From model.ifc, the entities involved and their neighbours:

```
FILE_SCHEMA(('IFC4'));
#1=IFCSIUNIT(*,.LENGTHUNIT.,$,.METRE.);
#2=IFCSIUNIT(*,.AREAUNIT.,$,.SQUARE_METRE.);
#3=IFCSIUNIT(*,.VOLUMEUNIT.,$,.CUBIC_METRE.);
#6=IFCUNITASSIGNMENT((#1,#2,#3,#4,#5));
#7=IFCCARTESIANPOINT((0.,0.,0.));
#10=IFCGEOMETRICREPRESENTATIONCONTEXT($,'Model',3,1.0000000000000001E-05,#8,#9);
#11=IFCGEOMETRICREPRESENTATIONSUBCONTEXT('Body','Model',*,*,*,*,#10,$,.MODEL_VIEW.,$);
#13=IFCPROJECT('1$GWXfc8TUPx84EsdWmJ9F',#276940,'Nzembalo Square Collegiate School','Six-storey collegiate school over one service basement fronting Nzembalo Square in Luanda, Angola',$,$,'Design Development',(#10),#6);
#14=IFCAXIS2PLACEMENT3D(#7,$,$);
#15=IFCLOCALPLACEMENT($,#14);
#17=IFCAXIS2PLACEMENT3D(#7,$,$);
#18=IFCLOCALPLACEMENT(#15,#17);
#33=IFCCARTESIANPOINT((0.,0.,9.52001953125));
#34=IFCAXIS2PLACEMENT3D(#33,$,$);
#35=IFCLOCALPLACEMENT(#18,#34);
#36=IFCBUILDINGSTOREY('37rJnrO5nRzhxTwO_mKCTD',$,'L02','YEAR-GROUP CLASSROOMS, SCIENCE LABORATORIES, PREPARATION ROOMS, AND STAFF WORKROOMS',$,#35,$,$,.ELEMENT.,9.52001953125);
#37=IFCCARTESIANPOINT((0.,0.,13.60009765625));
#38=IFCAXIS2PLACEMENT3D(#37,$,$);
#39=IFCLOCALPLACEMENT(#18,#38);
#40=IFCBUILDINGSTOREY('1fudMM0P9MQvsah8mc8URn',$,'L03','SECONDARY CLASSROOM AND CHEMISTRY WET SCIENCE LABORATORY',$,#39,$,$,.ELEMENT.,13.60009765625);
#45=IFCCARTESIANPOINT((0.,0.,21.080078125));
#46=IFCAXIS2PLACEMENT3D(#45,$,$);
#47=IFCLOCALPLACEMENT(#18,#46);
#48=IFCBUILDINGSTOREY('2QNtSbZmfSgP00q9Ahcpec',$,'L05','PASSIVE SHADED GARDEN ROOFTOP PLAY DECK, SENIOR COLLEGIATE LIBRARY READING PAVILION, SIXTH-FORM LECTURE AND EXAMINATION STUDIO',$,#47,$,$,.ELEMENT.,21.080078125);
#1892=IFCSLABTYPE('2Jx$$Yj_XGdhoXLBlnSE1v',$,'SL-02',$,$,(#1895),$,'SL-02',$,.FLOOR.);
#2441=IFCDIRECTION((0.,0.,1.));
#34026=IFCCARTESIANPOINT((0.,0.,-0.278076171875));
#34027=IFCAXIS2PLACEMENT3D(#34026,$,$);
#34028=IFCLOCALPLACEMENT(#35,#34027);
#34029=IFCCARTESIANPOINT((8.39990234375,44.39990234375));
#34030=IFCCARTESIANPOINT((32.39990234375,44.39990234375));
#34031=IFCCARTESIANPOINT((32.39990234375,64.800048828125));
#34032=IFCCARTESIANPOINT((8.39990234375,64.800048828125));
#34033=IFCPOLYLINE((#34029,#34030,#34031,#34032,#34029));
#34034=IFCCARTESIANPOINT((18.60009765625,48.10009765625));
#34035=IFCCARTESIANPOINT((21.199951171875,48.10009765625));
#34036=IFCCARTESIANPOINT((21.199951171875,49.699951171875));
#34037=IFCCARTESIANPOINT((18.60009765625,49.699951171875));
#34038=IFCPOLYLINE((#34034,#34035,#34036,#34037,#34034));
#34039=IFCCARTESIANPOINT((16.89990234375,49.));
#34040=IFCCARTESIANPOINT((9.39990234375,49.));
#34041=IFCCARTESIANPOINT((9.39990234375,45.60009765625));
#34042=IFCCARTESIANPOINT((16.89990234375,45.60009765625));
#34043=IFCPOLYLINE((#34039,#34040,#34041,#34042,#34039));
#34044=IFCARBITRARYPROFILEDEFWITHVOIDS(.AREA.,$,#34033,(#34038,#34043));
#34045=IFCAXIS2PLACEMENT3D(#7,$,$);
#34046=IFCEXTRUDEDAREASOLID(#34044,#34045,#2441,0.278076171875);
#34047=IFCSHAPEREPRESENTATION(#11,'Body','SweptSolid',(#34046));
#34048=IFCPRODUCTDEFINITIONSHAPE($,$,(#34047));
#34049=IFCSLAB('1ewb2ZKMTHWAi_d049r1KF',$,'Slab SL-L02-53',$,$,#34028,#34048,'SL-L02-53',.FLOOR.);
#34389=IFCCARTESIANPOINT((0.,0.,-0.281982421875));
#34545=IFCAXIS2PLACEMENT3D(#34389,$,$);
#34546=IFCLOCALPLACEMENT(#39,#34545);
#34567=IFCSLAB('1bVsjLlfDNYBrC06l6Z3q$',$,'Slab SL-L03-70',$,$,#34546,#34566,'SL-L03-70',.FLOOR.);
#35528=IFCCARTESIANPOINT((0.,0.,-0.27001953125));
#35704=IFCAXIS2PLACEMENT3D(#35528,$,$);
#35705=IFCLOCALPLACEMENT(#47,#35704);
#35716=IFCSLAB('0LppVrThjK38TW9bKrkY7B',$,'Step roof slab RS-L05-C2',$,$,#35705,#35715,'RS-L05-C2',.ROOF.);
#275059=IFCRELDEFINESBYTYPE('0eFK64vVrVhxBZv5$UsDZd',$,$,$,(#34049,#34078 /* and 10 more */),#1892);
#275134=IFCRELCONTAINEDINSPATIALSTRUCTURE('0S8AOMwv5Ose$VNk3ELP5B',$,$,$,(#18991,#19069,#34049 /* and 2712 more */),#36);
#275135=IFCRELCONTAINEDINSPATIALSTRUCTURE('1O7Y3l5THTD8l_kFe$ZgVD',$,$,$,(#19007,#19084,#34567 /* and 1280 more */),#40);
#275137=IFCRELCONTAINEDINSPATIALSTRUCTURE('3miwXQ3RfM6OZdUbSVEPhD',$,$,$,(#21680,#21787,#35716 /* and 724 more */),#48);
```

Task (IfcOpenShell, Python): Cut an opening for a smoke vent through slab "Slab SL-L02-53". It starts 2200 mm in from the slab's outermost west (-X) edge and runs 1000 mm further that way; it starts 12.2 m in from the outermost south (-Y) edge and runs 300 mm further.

```python
import numpy as np
import ifcopenshell
import ifcopenshell.api.feature
import ifcopenshell.api.geometry
import ifcopenshell.api.root
import ifcopenshell.geom
import ifcopenshell.util.placement
import ifcopenshell.util.representation
import ifcopenshell.util.shape
import ifcopenshell.util.unit

model = ifcopenshell.open("model.ifc")
unit_scale = ifcopenshell.util.unit.calculate_unit_scale(model)
settings = ifcopenshell.geom.settings()


def volume(element):
    """Net volume in cubic metres, openings subtracted."""
    shape = ifcopenshell.geom.create_shape(settings, element)
    return ifcopenshell.util.shape.get_volume(shape.geometry)


slab = model.by_id(34049)
before = volume(slab)

# Extent in the slab's own axes, in metres. The edges named are its -X and -Y sides.
slab_shape = ifcopenshell.geom.create_shape(settings, slab)
vertices = ifcopenshell.util.shape.get_vertices(slab_shape.geometry)
x_min, y_min, bottom = vertices.min(axis=0)
top = vertices[:, 2].max()

opening = ifcopenshell.api.root.create_entity(model, ifc_class="IfcOpeningElement", name="Smoke vent opening", predefined_type="OPENING")
context = ifcopenshell.util.representation.get_context(model, "Model", "Body", "MODEL_VIEW")
width, depth = 1, 0.3
outline = [(0.0, 0.0), (width, 0.0), (width, depth), (0.0, depth), (0.0, 0.0)]
# Overshoot both faces by 50 mm so the cut is clean.
shape = ifcopenshell.api.geometry.add_slab_representation(
    model, context=context, depth=top - bottom + 0.1, polyline=outline
)
ifcopenshell.api.geometry.assign_representation(model, product=opening, representation=shape)

matrix = ifcopenshell.util.placement.get_local_placement(slab.ObjectPlacement)
matrix[:, 3] = matrix @ np.append(np.array([x_min + 2.2, y_min + 12.2, bottom - 0.05]) / unit_scale, 1.0)
ifcopenshell.api.geometry.edit_object_placement(model, product=opening, matrix=matrix, is_si=False)
ifcopenshell.api.feature.add_feature(model, feature=opening, element=slab)

after = volume(slab)

print(f"slab volume {before:.3f} -> {after:.3f} m3")

model.write("model_updated.ifc")
```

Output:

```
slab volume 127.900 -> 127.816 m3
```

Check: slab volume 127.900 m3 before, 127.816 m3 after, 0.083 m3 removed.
